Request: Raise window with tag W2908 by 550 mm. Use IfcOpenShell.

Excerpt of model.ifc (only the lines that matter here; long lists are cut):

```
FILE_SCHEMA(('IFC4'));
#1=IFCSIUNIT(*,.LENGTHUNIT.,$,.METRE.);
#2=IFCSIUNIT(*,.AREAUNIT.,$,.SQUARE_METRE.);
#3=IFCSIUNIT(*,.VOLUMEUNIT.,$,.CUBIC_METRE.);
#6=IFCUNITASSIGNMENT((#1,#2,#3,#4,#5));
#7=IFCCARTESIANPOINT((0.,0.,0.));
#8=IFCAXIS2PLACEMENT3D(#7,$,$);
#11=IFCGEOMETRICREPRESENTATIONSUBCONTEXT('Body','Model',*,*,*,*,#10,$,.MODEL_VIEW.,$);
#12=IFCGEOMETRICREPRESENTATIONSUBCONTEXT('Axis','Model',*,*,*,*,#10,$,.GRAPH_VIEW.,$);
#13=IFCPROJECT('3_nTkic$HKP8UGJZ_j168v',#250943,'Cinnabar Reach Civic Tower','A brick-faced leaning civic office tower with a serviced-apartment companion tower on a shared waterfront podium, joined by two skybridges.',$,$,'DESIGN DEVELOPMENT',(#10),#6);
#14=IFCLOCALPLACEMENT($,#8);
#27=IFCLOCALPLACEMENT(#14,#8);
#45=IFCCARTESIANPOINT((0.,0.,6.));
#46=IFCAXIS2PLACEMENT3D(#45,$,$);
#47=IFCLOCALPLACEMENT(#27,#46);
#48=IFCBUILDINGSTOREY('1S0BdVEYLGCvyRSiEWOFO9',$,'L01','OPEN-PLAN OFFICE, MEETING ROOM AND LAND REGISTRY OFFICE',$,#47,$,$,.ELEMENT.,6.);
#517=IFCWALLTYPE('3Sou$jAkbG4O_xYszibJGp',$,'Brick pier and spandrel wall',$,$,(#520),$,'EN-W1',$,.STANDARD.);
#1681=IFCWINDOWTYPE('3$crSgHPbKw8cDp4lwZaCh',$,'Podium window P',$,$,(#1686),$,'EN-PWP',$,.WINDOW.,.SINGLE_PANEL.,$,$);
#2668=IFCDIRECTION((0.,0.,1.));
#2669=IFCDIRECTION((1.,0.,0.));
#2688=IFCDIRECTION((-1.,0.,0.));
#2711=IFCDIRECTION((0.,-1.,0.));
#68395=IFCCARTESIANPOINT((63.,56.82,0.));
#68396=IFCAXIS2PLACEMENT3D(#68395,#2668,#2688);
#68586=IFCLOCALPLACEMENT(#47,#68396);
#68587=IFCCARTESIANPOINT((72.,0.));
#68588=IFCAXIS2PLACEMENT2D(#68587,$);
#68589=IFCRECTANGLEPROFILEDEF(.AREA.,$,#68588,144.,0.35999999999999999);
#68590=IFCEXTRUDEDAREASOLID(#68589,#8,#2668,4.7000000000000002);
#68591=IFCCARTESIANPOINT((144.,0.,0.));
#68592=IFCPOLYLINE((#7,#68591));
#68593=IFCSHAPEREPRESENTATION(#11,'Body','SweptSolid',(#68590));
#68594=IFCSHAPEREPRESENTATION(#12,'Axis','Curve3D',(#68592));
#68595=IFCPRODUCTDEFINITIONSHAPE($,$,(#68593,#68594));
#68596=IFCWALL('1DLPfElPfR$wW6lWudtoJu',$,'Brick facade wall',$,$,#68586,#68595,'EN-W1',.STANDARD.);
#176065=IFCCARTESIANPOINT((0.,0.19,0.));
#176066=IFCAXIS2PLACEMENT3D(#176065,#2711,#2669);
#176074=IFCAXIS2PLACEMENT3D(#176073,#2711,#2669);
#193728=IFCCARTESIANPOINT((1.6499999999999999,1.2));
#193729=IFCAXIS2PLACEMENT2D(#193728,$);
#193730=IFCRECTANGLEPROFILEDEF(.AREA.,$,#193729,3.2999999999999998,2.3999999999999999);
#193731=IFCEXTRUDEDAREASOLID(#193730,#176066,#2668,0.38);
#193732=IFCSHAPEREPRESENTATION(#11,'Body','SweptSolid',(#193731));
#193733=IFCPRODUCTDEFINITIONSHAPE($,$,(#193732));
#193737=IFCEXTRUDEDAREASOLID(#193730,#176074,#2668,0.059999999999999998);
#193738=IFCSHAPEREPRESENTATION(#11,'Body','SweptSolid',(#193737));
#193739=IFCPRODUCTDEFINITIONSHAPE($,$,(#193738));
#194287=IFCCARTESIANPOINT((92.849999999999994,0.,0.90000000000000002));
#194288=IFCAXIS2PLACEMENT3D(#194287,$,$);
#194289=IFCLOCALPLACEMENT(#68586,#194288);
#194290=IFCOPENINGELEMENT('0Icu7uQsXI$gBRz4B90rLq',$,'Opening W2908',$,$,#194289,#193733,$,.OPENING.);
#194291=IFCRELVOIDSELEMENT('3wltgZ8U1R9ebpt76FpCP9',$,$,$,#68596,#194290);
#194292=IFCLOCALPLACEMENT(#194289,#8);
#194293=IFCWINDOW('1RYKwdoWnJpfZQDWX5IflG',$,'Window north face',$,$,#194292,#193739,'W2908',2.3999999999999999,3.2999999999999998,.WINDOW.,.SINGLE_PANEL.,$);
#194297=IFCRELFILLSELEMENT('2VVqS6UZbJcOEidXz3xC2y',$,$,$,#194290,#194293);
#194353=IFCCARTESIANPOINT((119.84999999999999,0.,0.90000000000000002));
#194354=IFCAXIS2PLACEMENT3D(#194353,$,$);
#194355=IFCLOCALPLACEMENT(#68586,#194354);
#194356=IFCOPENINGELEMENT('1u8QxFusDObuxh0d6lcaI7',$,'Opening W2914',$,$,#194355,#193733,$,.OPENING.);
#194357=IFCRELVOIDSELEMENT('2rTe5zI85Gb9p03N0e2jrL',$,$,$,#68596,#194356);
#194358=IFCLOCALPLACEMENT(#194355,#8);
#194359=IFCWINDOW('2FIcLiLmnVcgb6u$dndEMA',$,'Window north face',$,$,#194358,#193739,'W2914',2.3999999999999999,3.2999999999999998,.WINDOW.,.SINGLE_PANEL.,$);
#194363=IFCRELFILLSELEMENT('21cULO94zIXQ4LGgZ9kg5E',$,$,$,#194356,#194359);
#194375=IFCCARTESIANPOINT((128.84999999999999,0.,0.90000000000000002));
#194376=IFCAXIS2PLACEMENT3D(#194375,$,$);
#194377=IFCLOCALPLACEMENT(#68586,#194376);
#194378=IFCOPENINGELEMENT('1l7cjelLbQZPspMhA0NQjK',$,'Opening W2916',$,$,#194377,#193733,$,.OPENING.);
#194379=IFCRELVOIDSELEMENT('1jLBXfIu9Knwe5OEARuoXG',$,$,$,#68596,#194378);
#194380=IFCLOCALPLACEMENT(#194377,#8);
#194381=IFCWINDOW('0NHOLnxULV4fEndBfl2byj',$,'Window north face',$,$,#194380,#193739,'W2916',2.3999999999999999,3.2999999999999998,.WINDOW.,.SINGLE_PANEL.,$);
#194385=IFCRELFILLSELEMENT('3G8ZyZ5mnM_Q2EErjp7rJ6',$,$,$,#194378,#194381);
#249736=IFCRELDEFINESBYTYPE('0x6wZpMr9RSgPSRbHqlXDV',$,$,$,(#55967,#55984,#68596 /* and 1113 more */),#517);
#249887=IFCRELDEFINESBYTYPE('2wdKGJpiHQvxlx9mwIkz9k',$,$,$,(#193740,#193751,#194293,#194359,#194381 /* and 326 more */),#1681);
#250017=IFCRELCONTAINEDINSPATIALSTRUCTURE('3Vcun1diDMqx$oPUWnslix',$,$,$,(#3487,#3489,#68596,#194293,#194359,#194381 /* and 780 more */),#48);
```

```python
import numpy as np
import ifcopenshell
import ifcopenshell.api.geometry
import ifcopenshell.util.placement
import ifcopenshell.util.unit

model = ifcopenshell.open("model.ifc")
unit_scale = ifcopenshell.util.unit.calculate_unit_scale(model)

window = model.by_id(194293)
opening = window.FillsVoids[0].RelatingOpeningElement
dz = 0.55 / unit_scale

shift = np.array([0.0, 0.0, dz])
# The window is placed relative to its opening, so it follows when the opening moves.
matrix = ifcopenshell.util.placement.get_local_placement(opening.ObjectPlacement)
matrix[:3, 3] += shift
ifcopenshell.api.geometry.edit_object_placement(
    model, product=opening, matrix=matrix, is_si=False, should_transform_children=True
)

print(f"moved by {dz * unit_scale:+.3f} m")

model.write("model_rev.ifc")
```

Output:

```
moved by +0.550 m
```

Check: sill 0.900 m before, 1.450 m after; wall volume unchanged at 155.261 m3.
